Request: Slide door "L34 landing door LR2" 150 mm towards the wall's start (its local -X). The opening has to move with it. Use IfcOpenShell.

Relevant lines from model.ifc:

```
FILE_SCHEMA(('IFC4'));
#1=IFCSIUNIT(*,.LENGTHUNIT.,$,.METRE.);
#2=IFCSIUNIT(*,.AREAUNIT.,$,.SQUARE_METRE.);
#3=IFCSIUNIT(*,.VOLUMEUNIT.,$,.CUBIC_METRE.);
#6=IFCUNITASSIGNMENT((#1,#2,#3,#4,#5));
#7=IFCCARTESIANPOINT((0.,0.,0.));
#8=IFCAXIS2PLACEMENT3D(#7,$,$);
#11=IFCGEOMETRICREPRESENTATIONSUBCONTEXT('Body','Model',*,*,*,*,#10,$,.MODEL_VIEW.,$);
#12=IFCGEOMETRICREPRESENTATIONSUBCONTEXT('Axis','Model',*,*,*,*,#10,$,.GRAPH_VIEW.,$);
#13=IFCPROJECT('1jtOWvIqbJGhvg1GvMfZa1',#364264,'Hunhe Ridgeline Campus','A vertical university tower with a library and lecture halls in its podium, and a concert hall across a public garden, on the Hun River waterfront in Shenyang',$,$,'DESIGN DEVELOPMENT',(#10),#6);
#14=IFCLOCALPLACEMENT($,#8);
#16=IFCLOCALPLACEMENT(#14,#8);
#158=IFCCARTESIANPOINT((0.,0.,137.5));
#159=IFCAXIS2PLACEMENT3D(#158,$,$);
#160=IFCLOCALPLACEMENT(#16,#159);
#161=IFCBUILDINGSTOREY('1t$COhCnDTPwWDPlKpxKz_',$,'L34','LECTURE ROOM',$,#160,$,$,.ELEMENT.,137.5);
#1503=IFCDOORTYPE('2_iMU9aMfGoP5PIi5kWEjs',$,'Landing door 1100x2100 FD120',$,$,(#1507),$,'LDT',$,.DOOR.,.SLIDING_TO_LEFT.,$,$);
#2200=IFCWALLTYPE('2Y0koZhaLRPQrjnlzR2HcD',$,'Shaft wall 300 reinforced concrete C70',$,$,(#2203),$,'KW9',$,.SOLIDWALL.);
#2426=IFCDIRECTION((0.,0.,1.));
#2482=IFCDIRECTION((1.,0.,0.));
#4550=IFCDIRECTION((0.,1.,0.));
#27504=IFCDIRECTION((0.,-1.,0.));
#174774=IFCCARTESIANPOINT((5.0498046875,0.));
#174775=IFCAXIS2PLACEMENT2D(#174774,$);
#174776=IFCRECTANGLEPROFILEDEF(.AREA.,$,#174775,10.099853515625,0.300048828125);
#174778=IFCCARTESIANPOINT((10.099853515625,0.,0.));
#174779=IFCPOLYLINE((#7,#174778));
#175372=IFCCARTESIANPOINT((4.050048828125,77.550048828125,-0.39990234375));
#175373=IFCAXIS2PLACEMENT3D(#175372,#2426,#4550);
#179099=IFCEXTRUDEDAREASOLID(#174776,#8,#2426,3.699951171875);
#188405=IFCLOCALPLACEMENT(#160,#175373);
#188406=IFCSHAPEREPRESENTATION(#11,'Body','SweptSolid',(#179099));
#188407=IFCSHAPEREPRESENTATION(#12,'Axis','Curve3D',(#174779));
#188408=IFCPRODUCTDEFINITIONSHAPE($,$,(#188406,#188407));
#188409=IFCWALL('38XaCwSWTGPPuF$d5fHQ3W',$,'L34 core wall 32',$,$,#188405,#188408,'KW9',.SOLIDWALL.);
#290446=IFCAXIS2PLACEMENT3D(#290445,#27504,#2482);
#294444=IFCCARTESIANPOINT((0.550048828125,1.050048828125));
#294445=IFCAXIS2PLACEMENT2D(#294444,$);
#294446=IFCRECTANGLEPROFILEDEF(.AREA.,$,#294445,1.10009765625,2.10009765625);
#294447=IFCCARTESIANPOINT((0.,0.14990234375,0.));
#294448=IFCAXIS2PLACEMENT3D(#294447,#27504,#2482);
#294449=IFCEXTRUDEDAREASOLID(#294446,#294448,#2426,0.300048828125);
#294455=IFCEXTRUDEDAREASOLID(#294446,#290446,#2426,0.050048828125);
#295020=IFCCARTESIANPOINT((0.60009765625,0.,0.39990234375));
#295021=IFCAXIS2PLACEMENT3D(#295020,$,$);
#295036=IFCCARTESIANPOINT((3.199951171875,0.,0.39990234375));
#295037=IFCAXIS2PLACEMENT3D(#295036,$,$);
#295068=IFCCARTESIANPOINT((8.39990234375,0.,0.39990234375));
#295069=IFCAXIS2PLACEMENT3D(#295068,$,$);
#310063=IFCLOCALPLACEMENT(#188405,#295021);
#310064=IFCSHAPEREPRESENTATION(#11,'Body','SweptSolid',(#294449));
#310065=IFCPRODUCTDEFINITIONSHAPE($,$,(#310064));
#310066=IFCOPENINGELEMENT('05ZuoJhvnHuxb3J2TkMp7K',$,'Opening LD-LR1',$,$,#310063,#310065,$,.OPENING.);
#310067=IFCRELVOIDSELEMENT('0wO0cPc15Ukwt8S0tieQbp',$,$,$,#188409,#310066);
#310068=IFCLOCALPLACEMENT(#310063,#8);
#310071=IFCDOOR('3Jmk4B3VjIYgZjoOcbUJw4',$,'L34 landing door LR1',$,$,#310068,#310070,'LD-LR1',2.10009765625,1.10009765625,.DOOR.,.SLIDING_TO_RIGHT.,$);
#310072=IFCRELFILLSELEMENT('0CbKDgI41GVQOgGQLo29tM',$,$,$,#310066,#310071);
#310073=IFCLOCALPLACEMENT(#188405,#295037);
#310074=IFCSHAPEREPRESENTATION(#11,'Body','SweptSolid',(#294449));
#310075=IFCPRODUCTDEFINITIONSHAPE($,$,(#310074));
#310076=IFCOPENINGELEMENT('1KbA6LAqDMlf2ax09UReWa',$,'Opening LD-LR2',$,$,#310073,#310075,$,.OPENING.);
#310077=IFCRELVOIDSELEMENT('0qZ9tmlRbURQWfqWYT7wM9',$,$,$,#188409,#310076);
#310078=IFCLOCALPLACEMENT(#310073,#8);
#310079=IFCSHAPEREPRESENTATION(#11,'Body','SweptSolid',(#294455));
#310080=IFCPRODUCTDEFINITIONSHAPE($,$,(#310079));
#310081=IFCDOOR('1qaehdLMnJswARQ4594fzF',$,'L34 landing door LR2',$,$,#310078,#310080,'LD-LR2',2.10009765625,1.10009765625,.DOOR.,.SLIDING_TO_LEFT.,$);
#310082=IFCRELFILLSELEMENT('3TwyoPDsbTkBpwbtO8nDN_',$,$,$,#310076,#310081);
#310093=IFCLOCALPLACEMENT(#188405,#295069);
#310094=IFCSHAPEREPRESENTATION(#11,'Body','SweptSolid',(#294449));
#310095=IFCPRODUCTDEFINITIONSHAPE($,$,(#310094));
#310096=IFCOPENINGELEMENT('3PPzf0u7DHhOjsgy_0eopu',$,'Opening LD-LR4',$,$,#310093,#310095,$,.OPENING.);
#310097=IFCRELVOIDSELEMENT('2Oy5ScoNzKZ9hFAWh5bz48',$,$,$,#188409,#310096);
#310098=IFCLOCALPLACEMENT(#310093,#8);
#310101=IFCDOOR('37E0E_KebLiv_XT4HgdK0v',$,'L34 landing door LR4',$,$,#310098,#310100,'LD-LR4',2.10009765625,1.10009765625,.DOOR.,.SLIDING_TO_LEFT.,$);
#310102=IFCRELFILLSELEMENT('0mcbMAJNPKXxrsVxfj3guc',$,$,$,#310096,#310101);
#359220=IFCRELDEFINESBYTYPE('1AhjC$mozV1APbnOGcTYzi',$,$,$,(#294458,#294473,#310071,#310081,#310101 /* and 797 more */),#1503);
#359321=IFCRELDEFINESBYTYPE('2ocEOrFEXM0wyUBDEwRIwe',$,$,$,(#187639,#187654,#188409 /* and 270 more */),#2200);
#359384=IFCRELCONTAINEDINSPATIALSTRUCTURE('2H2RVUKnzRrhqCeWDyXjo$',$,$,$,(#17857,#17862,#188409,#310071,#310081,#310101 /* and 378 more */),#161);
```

```python
import ifcopenshell
import ifcopenshell.api.geometry
import ifcopenshell.util.placement
import ifcopenshell.util.unit

model = ifcopenshell.open("model.ifc")
unit_scale = ifcopenshell.util.unit.calculate_unit_scale(model)

door = model.by_guid("1qaehdLMnJswARQ4594fzF")
opening = door.FillsVoids[0].RelatingOpeningElement
wall = opening.VoidsElements[0].RelatingBuildingElement

wall_matrix = ifcopenshell.util.placement.get_local_placement(wall.ObjectPlacement)
shift = wall_matrix[:3, 0] * -0.15 / unit_scale
before = ifcopenshell.util.placement.get_local_placement(door.ObjectPlacement)[:3, 3].copy()

# The door is placed relative to its opening, so it follows when the opening moves.
matrix = ifcopenshell.util.placement.get_local_placement(opening.ObjectPlacement)
matrix[:3, 3] += shift
ifcopenshell.api.geometry.edit_object_placement(
    model, product=opening, matrix=matrix, is_si=False, should_transform_children=True
)

after = ifcopenshell.util.placement.get_local_placement(door.ObjectPlacement)[:3, 3]
print("door moved by", (after - before).round(3) + 0.0)

model.write("model_edited.ifc")
```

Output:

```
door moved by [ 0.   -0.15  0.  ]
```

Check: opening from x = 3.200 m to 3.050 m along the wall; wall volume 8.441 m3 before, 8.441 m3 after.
